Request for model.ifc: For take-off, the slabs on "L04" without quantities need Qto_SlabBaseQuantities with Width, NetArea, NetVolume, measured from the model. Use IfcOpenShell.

First a look at what the model holds.

```python
import ifcopenshell
import ifcopenshell.util.element
import ifcopenshell.util.unit

model = ifcopenshell.open("model.ifc")
print(model.schema)
for unit_type in ("LENGTHUNIT", "AREAUNIT", "VOLUMEUNIT"):
    print(unit_type, ifcopenshell.util.unit.calculate_unit_scale(model, unit_type))
storey = next(s for s in model.by_type("IfcBuildingStorey") if s.Name == "L04")
slabs = [e for e in ifcopenshell.util.element.get_decomposition(storey) if e.is_a("IfcSlab")]
for e in sorted(slabs, key=lambda e: e.id()):
    print(e.id(), e.is_a(), e.Name, list(ifcopenshell.util.element.get_psets(e, qtos_only=True)), sep=" | ")
```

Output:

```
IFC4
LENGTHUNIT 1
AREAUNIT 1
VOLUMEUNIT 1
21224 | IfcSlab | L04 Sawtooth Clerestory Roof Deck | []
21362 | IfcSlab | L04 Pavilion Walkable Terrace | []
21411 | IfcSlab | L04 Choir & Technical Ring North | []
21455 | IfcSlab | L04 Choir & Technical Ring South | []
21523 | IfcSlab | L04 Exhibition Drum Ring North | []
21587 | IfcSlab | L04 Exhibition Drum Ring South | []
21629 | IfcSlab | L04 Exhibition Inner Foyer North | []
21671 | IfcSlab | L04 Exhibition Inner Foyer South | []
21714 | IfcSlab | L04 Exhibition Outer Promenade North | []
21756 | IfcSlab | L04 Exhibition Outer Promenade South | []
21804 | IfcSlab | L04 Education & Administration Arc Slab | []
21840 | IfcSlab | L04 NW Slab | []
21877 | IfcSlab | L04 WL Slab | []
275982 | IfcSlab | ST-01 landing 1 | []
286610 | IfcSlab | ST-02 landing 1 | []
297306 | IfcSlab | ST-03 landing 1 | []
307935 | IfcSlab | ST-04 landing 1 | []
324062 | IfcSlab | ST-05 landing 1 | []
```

```python
import ifcopenshell
import ifcopenshell.api.pset
import ifcopenshell.geom
import ifcopenshell.util.element
import ifcopenshell.util.shape
import ifcopenshell.util.unit

model = ifcopenshell.open("model.ifc")
unit_scale = ifcopenshell.util.unit.calculate_unit_scale(model)
area_scale = ifcopenshell.util.unit.calculate_unit_scale(model, "AREAUNIT")
volume_scale = ifcopenshell.util.unit.calculate_unit_scale(model, "VOLUMEUNIT")
settings = ifcopenshell.geom.settings()

storey = next(s for s in model.by_type("IfcBuildingStorey") if s.Name == "L04")
slabs = [e for e in ifcopenshell.util.element.get_decomposition(storey) if e.is_a("IfcSlab")]

for e in sorted(slabs, key=lambda e: e.id()):
    if ifcopenshell.util.element.get_psets(e, qtos_only=True, should_inherit=False):
        continue
    # Geometry comes back in metres, in the element's own axes.
    shape = ifcopenshell.geom.create_shape(settings, e)
    values = {
        "Width": ifcopenshell.util.shape.get_z(shape.geometry) / unit_scale,
        "NetArea": ifcopenshell.util.shape.get_footprint_area(shape.geometry) / area_scale,
        "NetVolume": ifcopenshell.util.shape.get_volume(shape.geometry) / volume_scale,
    }
    qto = ifcopenshell.api.pset.add_qto(model, product=e, name="Qto_SlabBaseQuantities")
    ifcopenshell.api.pset.edit_qto(model, qto=qto, properties=values)
    print(e.id(), {k: round(v, 3) for k, v in values.items()})

model.write("model-out.ifc")
```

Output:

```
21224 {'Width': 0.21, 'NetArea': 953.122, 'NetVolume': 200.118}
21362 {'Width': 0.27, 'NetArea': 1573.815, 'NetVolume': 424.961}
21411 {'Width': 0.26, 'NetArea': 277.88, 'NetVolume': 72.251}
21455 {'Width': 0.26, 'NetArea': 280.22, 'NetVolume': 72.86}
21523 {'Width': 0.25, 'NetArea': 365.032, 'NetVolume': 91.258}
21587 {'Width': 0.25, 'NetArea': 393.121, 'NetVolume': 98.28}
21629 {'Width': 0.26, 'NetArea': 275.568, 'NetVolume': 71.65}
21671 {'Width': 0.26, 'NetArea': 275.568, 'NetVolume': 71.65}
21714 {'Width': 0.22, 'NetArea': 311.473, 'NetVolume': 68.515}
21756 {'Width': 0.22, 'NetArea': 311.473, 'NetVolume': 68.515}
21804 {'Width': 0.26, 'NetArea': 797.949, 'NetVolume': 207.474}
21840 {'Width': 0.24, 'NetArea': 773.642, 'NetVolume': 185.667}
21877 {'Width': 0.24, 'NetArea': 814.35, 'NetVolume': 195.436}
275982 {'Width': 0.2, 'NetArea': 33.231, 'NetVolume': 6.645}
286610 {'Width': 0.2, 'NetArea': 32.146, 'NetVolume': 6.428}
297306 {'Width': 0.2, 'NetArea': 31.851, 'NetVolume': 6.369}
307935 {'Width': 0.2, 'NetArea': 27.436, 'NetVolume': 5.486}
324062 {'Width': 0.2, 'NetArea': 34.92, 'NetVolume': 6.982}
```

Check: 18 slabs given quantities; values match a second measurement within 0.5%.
